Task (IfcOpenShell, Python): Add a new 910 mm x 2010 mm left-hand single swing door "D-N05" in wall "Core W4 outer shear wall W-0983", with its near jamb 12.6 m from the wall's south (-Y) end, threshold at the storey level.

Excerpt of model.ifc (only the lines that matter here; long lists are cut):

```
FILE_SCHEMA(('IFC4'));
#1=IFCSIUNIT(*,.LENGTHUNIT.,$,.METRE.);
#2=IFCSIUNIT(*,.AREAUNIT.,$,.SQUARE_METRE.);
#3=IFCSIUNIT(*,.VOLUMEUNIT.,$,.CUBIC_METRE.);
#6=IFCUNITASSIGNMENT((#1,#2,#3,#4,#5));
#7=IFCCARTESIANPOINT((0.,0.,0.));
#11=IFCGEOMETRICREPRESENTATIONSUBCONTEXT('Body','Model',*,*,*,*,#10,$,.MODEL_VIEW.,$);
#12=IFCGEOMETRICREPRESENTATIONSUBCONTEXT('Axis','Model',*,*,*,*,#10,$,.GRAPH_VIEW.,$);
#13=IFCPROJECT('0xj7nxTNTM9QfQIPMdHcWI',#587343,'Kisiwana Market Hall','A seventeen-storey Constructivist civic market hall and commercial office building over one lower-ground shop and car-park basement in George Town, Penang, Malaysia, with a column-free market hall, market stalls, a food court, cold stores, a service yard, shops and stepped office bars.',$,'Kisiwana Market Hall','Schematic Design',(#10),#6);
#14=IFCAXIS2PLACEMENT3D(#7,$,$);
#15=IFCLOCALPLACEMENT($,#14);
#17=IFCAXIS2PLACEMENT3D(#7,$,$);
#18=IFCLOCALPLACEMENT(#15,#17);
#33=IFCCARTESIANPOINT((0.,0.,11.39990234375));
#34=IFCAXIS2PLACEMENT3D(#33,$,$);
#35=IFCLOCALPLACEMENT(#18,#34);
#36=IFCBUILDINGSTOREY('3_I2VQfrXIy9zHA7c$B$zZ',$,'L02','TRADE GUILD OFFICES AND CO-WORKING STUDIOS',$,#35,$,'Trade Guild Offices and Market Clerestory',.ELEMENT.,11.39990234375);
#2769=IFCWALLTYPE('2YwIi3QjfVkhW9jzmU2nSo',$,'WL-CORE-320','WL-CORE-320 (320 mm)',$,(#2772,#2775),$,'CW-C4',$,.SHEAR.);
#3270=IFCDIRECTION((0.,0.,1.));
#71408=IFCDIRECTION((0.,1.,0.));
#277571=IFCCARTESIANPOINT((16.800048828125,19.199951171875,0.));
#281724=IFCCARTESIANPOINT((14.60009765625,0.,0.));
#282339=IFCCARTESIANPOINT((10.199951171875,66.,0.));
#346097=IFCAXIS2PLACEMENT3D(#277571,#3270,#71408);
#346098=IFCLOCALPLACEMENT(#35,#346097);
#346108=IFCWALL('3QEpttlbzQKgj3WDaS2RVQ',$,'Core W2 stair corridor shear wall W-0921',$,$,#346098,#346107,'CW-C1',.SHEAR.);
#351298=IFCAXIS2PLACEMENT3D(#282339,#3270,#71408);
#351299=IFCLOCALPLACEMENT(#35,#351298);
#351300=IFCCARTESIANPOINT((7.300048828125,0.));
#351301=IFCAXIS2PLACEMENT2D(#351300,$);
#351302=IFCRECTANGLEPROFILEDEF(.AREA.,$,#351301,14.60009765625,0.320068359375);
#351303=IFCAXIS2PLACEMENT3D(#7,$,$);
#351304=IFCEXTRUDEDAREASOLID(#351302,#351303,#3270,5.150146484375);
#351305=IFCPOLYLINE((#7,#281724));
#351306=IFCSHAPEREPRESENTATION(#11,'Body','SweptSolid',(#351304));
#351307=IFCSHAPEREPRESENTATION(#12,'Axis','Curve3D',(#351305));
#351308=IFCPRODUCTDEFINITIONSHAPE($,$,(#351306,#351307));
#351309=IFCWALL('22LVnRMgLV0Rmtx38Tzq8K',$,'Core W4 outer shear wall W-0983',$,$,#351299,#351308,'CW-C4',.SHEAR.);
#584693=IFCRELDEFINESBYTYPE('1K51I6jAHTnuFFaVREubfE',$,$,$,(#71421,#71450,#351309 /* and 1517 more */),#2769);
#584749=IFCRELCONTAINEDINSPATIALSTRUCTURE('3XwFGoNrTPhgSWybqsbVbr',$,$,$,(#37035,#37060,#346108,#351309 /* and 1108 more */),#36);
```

```python
import numpy as np
import ifcopenshell
import ifcopenshell.api.feature
import ifcopenshell.api.geometry
import ifcopenshell.api.root
import ifcopenshell.api.spatial
import ifcopenshell.geom
import ifcopenshell.util.element
import ifcopenshell.util.placement
import ifcopenshell.util.representation
import ifcopenshell.util.shape
import ifcopenshell.util.unit

model = ifcopenshell.open("model.ifc")
unit_scale = ifcopenshell.util.unit.calculate_unit_scale(model)
settings = ifcopenshell.geom.settings()


def volume(element):
    """Net volume in cubic metres, openings subtracted."""
    shape = ifcopenshell.geom.create_shape(settings, element)
    return ifcopenshell.util.shape.get_volume(shape.geometry)


wall = model.by_guid("22LVnRMgLV0Rmtx38Tzq8K")
storey = ifcopenshell.util.element.get_container(wall, ifc_class="IfcBuildingStorey")
context = ifcopenshell.util.representation.get_context(model, "Model", "Body", "MODEL_VIEW")
before = volume(wall)

width, height, from_end, sill = 0.91, 2.01, 12.6, 0.0  # metres

# The wall runs along its own X axis, and the end named is its -X end.
wall_shape = ifcopenshell.geom.create_shape(settings, wall)
x, y, z = ifcopenshell.util.shape.get_vertices(wall_shape.geometry).T
start = x.min() + from_end
face, thickness = float(y.min()), float(y.max() - y.min())
wall_matrix = ifcopenshell.util.placement.get_local_placement(wall.ObjectPlacement)
level = ifcopenshell.util.placement.get_local_placement(storey.ObjectPlacement)[2, 3]


def in_wall(x, y):
    """Placement at x, y metres in the wall's axes, at sill height."""
    matrix = wall_matrix.copy()
    matrix[:, 3] = wall_matrix @ np.array([x / unit_scale, y / unit_scale, 0.0, 1.0])
    matrix[2, 3] = level + sill / unit_scale
    return matrix


# Opening: a box that overshoots both wall faces by 50 mm.
opening = ifcopenshell.api.root.create_entity(model, ifc_class="IfcOpeningElement", predefined_type="OPENING")
box = ifcopenshell.api.geometry.add_wall_representation(
    model, context=context, length=width, height=height, thickness=thickness + 0.1
)
ifcopenshell.api.geometry.assign_representation(model, product=opening, representation=box)
ifcopenshell.api.geometry.edit_object_placement(model, product=opening, matrix=in_wall(start, face - 0.05), is_si=False)
ifcopenshell.api.feature.add_feature(model, feature=opening, element=wall)

door = ifcopenshell.api.root.create_entity(model, ifc_class="IfcDoor", name="D-N05", predefined_type="DOOR")
door.OverallWidth, door.OverallHeight = width / unit_scale, height / unit_scale
door.OperationType = "SINGLE_SWING_LEFT"
body = ifcopenshell.api.geometry.add_door_representation(
    model,
    context=context,
    overall_width=door.OverallWidth,
    overall_height=door.OverallHeight,
    operation_type="SINGLE_SWING_LEFT",
    lining_properties={"LiningDepth": thickness / unit_scale, "ThresholdDepth": thickness / unit_scale},
)
ifcopenshell.api.geometry.assign_representation(model, product=door, representation=body)
ifcopenshell.api.spatial.assign_container(model, products=[door], relating_structure=storey)
ifcopenshell.api.feature.add_filling(model, opening=opening, element=door)

# The lining spans the wall, so the door starts at the wall face.
ifcopenshell.api.geometry.edit_object_placement(model, product=door, matrix=in_wall(start, face), is_si=False)

after = volume(wall)

print(f"wall volume {before:.3f} -> {after:.3f} m3")

model.write("model_v2.ifc")
```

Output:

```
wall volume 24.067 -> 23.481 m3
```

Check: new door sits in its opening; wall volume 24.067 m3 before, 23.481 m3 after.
